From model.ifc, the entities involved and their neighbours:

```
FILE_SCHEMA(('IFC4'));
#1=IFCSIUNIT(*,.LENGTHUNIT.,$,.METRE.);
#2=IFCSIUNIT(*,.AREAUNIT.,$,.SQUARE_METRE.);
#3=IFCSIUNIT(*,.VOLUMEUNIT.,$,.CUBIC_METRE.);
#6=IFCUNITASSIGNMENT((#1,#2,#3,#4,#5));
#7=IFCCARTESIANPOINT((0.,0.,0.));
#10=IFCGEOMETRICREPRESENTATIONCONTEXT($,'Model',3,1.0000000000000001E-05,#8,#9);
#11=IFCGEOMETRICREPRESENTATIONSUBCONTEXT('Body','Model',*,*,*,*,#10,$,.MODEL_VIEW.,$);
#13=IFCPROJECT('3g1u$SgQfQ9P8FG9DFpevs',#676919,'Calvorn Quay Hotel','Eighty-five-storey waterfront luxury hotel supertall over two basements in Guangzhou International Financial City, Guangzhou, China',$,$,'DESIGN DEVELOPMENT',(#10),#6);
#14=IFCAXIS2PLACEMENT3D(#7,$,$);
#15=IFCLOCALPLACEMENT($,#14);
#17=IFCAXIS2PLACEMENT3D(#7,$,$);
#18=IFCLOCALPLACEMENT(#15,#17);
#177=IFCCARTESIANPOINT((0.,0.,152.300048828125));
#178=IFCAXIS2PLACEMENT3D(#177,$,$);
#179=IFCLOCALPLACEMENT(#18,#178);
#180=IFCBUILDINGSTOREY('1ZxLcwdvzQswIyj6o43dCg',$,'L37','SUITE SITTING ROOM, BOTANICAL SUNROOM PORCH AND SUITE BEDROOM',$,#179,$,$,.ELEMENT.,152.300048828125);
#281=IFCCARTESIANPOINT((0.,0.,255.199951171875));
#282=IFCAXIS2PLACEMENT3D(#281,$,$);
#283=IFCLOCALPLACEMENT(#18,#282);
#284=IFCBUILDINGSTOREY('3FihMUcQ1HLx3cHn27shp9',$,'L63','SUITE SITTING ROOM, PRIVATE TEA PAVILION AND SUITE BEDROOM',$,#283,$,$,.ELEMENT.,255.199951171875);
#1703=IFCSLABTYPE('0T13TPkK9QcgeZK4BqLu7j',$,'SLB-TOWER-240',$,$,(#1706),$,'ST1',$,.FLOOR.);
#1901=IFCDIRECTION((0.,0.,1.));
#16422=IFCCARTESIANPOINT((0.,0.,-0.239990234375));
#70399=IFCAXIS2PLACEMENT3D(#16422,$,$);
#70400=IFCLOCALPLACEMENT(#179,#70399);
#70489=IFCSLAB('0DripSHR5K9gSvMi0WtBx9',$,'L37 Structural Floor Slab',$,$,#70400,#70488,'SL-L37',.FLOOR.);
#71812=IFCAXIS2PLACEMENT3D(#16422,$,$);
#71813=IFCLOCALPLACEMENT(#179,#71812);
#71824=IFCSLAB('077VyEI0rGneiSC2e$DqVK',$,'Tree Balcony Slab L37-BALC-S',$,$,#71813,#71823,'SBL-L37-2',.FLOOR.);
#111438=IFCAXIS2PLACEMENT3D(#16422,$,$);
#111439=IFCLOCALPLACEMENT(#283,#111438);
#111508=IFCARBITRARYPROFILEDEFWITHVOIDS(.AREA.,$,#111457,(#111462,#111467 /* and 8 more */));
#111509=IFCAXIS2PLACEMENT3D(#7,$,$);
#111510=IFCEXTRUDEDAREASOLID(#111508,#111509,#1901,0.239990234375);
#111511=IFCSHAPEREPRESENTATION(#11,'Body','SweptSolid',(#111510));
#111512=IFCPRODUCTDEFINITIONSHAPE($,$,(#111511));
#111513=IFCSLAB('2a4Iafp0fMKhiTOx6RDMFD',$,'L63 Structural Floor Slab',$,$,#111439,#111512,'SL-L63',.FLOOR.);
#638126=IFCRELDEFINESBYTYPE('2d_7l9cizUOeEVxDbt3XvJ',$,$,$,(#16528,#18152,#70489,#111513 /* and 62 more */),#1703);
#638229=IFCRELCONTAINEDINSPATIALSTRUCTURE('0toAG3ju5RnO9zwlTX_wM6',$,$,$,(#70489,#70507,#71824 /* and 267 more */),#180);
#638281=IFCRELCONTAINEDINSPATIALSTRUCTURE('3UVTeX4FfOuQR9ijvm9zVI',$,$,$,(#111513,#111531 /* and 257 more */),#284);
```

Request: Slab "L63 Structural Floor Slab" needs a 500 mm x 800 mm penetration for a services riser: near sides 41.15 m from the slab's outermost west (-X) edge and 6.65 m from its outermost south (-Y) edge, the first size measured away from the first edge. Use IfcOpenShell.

```python
import numpy as np
import ifcopenshell
import ifcopenshell.api.feature
import ifcopenshell.api.geometry
import ifcopenshell.api.root
import ifcopenshell.geom
import ifcopenshell.util.placement
import ifcopenshell.util.representation
import ifcopenshell.util.shape
import ifcopenshell.util.unit

model = ifcopenshell.open("model.ifc")
unit_scale = ifcopenshell.util.unit.calculate_unit_scale(model)
settings = ifcopenshell.geom.settings()


def volume(element):
    """Net volume in cubic metres, openings subtracted."""
    shape = ifcopenshell.geom.create_shape(settings, element)
    return ifcopenshell.util.shape.get_volume(shape.geometry)


slab = model.by_guid("2a4Iafp0fMKhiTOx6RDMFD")
before = volume(slab)

# Extent in the slab's own axes, in metres. The edges named are its -X and -Y sides.
slab_shape = ifcopenshell.geom.create_shape(settings, slab)
vertices = ifcopenshell.util.shape.get_vertices(slab_shape.geometry)
x_min, y_min, bottom = vertices.min(axis=0)
top = vertices[:, 2].max()

opening = ifcopenshell.api.root.create_entity(model, ifc_class="IfcOpeningElement", name="Services riser opening", predefined_type="OPENING")
context = ifcopenshell.util.representation.get_context(model, "Model", "Body", "MODEL_VIEW")
width, depth = 0.5, 0.8
outline = [(0.0, 0.0), (width, 0.0), (width, depth), (0.0, depth), (0.0, 0.0)]
# Overshoot both faces by 50 mm so the cut is clean.
shape = ifcopenshell.api.geometry.add_slab_representation(
    model, context=context, depth=top - bottom + 0.1, polyline=outline
)
ifcopenshell.api.geometry.assign_representation(model, product=opening, representation=shape)

matrix = ifcopenshell.util.placement.get_local_placement(slab.ObjectPlacement)
matrix[:, 3] = matrix @ np.append(np.array([x_min + 41.15, y_min + 6.65, bottom - 0.05]) / unit_scale, 1.0)
ifcopenshell.api.geometry.edit_object_placement(model, product=opening, matrix=matrix, is_si=False)
ifcopenshell.api.feature.add_feature(model, feature=opening, element=slab)

after = volume(slab)

print(f"slab volume {before:.3f} -> {after:.3f} m3")

model.write("model_edited.ifc")
```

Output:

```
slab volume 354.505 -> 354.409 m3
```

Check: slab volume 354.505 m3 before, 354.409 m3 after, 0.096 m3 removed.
